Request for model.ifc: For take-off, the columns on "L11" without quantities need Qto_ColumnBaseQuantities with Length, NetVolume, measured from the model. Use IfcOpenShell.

First a look at what the model holds.

```python
import ifcopenshell
import ifcopenshell.util.element
import ifcopenshell.util.unit

model = ifcopenshell.open("model.ifc")
print(model.schema)
for unit_type in ("LENGTHUNIT", "AREAUNIT", "VOLUMEUNIT"):
    print(unit_type, ifcopenshell.util.unit.calculate_unit_scale(model, unit_type))
storey = next(s for s in model.by_type("IfcBuildingStorey") if s.Name == "L11")
columns = [e for e in ifcopenshell.util.element.get_decomposition(storey) if e.is_a("IfcColumn")]
for e in sorted(columns, key=lambda e: e.id()):
    print(e.id(), e.is_a(), e.Name, list(ifcopenshell.util.element.get_psets(e, qtos_only=True)), sep=" | ")
```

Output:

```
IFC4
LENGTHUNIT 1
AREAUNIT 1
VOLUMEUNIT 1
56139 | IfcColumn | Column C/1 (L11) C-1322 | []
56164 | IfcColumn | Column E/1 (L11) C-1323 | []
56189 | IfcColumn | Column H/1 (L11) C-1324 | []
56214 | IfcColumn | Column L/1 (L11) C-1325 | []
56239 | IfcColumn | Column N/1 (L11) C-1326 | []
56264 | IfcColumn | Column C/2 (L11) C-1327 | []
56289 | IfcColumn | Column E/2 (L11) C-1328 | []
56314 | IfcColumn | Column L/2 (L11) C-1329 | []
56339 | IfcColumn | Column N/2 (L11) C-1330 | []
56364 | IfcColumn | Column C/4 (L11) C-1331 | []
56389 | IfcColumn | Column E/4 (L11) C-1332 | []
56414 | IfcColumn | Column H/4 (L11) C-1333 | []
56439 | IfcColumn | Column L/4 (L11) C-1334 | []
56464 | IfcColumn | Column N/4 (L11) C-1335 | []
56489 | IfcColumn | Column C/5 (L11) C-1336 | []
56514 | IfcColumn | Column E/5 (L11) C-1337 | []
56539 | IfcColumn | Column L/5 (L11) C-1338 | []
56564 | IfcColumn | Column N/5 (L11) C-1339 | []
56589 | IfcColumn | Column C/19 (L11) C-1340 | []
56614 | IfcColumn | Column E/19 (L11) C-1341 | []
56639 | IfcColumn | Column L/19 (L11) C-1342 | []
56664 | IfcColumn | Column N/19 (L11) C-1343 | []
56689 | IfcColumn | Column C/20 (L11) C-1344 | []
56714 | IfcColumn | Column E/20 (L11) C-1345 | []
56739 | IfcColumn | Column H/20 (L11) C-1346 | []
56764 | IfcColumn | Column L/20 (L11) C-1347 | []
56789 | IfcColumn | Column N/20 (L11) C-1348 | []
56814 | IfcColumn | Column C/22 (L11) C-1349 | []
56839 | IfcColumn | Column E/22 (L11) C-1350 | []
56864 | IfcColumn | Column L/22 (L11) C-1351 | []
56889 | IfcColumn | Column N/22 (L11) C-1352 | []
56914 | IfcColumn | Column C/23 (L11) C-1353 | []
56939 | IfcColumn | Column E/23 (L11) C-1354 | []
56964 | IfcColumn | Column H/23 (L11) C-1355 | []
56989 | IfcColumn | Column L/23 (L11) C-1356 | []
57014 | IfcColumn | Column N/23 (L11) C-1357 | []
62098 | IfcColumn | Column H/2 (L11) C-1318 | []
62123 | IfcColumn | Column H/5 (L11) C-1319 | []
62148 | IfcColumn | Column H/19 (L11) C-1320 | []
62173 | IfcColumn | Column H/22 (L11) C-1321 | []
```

```python
import ifcopenshell
import ifcopenshell.api.pset
import ifcopenshell.geom
import ifcopenshell.util.element
import ifcopenshell.util.shape
import ifcopenshell.util.unit

model = ifcopenshell.open("model.ifc")
unit_scale = ifcopenshell.util.unit.calculate_unit_scale(model)
volume_scale = ifcopenshell.util.unit.calculate_unit_scale(model, "VOLUMEUNIT")
settings = ifcopenshell.geom.settings()

storey = next(s for s in model.by_type("IfcBuildingStorey") if s.Name == "L11")
columns = [e for e in ifcopenshell.util.element.get_decomposition(storey) if e.is_a("IfcColumn")]

for e in sorted(columns, key=lambda e: e.id()):
    if ifcopenshell.util.element.get_psets(e, qtos_only=True, should_inherit=False):
        continue
    # Geometry comes back in metres, in the element's own axes.
    shape = ifcopenshell.geom.create_shape(settings, e)
    values = {
        "Length": ifcopenshell.util.shape.get_z(shape.geometry) / unit_scale,
        "NetVolume": ifcopenshell.util.shape.get_volume(shape.geometry) / volume_scale,
    }
    qto = ifcopenshell.api.pset.add_qto(model, product=e, name="Qto_ColumnBaseQuantities")
    ifcopenshell.api.pset.edit_qto(model, qto=qto, properties=values)
    print(e.id(), {k: round(v, 3) for k, v in values.items()})

model.write("model_v2.ifc")
```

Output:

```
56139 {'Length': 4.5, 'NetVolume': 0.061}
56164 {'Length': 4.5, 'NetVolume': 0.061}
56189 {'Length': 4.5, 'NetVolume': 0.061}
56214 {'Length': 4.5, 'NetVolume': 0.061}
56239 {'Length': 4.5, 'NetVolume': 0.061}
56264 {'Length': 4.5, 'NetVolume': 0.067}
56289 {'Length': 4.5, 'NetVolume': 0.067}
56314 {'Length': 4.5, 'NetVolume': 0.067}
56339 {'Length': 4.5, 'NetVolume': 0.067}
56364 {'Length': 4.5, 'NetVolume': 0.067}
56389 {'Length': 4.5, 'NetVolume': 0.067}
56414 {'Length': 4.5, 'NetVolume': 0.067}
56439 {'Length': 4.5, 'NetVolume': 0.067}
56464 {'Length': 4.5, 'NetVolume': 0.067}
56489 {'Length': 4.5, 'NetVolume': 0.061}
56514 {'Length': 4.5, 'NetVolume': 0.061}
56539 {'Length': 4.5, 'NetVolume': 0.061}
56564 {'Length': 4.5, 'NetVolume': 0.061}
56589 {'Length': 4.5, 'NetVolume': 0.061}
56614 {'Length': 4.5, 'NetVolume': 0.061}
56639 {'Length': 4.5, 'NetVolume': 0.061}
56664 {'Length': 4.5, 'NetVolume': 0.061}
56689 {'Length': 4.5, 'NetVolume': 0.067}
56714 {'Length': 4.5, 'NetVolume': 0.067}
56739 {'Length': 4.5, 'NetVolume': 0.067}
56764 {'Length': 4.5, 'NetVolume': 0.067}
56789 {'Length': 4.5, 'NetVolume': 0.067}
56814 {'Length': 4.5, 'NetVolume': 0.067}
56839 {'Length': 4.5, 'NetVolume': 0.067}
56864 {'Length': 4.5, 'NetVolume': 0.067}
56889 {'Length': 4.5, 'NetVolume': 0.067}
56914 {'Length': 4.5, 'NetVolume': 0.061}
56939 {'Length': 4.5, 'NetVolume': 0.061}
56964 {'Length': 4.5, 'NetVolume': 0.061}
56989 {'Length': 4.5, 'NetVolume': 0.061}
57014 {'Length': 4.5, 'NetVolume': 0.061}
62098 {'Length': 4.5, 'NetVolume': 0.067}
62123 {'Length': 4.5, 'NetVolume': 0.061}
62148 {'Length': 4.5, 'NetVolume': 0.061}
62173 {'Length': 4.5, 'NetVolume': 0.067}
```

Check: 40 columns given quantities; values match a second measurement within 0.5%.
